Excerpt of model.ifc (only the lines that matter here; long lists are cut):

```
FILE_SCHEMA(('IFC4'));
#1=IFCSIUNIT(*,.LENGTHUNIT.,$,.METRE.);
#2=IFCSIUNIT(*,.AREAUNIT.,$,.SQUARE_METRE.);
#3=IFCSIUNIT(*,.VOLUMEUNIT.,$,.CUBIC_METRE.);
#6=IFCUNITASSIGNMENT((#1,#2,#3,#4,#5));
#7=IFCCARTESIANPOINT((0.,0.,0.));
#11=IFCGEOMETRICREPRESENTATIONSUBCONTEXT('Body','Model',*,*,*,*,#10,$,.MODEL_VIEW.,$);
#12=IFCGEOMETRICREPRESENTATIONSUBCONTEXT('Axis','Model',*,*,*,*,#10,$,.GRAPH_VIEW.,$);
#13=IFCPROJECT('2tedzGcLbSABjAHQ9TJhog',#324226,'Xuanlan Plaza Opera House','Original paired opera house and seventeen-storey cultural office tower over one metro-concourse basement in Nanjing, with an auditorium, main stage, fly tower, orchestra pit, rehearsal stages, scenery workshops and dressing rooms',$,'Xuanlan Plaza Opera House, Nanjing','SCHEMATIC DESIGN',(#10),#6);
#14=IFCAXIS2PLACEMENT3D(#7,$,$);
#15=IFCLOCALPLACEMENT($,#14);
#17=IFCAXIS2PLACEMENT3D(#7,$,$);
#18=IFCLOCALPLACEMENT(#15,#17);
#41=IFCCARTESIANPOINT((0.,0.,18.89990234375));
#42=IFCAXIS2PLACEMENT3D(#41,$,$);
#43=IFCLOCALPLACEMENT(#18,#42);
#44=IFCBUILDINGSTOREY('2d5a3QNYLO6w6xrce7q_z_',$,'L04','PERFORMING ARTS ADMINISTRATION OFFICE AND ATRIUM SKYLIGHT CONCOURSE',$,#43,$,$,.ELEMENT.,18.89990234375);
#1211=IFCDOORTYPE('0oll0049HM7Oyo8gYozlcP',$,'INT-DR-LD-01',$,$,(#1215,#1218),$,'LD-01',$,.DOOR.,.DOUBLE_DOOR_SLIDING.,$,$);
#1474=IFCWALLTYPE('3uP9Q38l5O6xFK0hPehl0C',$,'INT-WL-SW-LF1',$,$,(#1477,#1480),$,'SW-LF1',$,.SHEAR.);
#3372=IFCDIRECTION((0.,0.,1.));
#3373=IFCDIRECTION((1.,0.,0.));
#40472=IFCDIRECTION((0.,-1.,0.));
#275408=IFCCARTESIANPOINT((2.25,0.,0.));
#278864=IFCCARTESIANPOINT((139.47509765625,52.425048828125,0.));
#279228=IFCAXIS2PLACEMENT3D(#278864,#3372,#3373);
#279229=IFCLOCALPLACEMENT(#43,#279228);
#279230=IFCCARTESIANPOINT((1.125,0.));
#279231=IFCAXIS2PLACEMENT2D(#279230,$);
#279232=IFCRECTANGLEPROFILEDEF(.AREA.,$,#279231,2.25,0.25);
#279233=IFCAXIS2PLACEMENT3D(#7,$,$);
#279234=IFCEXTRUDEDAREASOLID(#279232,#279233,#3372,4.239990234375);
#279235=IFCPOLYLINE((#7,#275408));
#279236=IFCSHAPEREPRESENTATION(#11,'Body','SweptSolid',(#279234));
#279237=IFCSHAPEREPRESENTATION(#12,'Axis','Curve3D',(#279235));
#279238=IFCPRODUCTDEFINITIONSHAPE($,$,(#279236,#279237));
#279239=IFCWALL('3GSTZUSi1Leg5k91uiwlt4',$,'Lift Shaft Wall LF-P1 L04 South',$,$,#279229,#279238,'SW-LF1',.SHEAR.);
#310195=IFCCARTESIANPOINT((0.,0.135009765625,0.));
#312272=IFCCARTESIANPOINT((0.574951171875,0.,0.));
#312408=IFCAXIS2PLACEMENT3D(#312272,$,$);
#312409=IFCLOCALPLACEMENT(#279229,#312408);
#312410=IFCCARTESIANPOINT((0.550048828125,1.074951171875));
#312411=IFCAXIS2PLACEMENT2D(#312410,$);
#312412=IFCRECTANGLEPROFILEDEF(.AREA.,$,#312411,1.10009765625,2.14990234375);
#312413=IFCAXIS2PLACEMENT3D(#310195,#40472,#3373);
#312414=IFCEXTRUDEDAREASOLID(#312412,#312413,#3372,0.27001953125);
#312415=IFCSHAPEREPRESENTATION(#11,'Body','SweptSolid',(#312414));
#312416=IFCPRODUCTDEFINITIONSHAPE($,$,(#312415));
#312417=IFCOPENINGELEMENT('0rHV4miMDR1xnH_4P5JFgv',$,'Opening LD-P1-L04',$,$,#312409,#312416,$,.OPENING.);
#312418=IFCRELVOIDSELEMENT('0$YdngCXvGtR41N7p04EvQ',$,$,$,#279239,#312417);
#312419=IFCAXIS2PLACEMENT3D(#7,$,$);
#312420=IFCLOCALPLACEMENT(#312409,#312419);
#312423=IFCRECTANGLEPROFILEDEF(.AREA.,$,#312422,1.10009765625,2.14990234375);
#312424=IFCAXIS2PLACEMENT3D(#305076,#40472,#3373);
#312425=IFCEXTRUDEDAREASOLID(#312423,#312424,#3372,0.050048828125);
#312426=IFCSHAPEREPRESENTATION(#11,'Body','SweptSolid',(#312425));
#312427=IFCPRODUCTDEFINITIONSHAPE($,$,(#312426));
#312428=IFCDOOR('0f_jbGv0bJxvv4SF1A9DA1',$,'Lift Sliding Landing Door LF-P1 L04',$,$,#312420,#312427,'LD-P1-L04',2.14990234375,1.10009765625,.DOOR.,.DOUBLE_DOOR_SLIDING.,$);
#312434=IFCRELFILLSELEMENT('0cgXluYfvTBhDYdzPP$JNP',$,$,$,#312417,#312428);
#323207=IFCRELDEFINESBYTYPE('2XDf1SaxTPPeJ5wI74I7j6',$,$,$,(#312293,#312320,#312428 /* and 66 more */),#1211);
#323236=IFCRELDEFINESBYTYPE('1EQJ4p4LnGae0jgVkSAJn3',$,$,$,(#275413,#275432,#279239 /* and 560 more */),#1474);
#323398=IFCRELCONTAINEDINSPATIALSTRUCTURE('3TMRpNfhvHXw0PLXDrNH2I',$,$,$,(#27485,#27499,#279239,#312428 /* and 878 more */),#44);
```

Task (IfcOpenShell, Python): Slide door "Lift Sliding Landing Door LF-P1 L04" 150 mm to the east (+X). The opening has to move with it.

```python
import ifcopenshell
import ifcopenshell.api.geometry
import ifcopenshell.util.placement

model = ifcopenshell.open("model.ifc")

door = model.by_guid("0f_jbGv0bJxvv4SF1A9DA1")
opening = door.FillsVoids[0].RelatingOpeningElement
wall = opening.VoidsElements[0].RelatingBuildingElement

wall_matrix = ifcopenshell.util.placement.get_local_placement(wall.ObjectPlacement)
shift = wall_matrix[:3, 0] * 0.15
before = ifcopenshell.util.placement.get_local_placement(door.ObjectPlacement)[:3, 3].copy()

# The door is placed relative to its opening, so it follows when the opening moves.
matrix = ifcopenshell.util.placement.get_local_placement(opening.ObjectPlacement)
matrix[:3, 3] += shift
ifcopenshell.api.geometry.edit_object_placement(
    model, product=opening, matrix=matrix, is_si=False, should_transform_children=True
)

after = ifcopenshell.util.placement.get_local_placement(door.ObjectPlacement)[:3, 3]
print("door moved by", (after - before).round(3) + 0.0)

model.write("model_edited.ifc")
```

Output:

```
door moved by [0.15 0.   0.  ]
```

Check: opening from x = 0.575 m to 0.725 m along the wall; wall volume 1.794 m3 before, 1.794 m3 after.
